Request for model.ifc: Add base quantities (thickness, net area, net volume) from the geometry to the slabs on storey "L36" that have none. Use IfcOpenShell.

First a look at what the model holds.

```python
import ifcopenshell
import ifcopenshell.util.element
import ifcopenshell.util.unit

model = ifcopenshell.open("model.ifc")
print(model.schema)
for unit_type in ("LENGTHUNIT", "AREAUNIT", "VOLUMEUNIT"):
    print(unit_type, ifcopenshell.util.unit.calculate_unit_scale(model, unit_type))
storey = next(s for s in model.by_type("IfcBuildingStorey") if s.Name == "L36")
slabs = [e for e in ifcopenshell.util.element.get_decomposition(storey) if e.is_a("IfcSlab")]
for e in sorted(slabs, key=lambda e: e.id()):
    print(e.id(), e.is_a(), e.Name, list(ifcopenshell.util.element.get_psets(e, qtos_only=True)), sep=" | ")
```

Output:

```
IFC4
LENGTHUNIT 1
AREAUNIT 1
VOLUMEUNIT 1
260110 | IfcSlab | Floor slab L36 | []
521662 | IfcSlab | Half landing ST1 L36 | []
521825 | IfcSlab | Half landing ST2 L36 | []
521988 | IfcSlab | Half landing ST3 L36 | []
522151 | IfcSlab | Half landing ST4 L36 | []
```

```python
import ifcopenshell
import ifcopenshell.api.pset
import ifcopenshell.geom
import ifcopenshell.util.element
import ifcopenshell.util.shape
import ifcopenshell.util.unit

model = ifcopenshell.open("model.ifc")
unit_scale = ifcopenshell.util.unit.calculate_unit_scale(model)
area_scale = ifcopenshell.util.unit.calculate_unit_scale(model, "AREAUNIT")
volume_scale = ifcopenshell.util.unit.calculate_unit_scale(model, "VOLUMEUNIT")
settings = ifcopenshell.geom.settings()

storey = next(s for s in model.by_type("IfcBuildingStorey") if s.Name == "L36")
slabs = [e for e in ifcopenshell.util.element.get_decomposition(storey) if e.is_a("IfcSlab")]

for e in sorted(slabs, key=lambda e: e.id()):
    if ifcopenshell.util.element.get_psets(e, qtos_only=True, should_inherit=False):
        continue
    # Geometry comes back in metres, in the element's own axes.
    shape = ifcopenshell.geom.create_shape(settings, e)
    values = {
        "Width": ifcopenshell.util.shape.get_z(shape.geometry) / unit_scale,
        "NetArea": ifcopenshell.util.shape.get_footprint_area(shape.geometry) / area_scale,
        "NetVolume": ifcopenshell.util.shape.get_volume(shape.geometry) / volume_scale,
    }
    qto = ifcopenshell.api.pset.add_qto(model, product=e, name="Qto_SlabBaseQuantities")
    ifcopenshell.api.pset.edit_qto(model, qto=qto, properties=values)
    print(e.id(), {k: round(v, 3) for k, v in values.items()})

model.write("model_updated.ifc")
```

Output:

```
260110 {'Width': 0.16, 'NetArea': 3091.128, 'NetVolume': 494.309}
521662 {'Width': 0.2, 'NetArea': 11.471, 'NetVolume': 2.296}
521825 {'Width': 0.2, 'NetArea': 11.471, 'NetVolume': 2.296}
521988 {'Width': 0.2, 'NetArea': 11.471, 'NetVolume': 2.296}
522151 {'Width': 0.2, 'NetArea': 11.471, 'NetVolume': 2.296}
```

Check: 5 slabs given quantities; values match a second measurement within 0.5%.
